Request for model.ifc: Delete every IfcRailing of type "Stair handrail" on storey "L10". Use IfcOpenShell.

First a look at what the model holds.

```python
import ifcopenshell
import ifcopenshell.util.element

model = ifcopenshell.open("model.ifc")
print(model.schema)
storey = next(s for s in model.by_type("IfcBuildingStorey") if s.Name == "L10")
railings = [e for e in ifcopenshell.util.element.get_decomposition(storey) if e.is_a("IfcRailing")]
seen = {}
for e in railings:
    element_type = ifcopenshell.util.element.get_type(e)
    name = element_type.Name if element_type not in (None, e) else None
    seen[name] = seen.get(name, 0) + 1
for name, count in sorted(seen.items(), key=str):
    print(count, "x", name)
```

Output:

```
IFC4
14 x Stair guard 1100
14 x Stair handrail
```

```python
import ifcopenshell
import ifcopenshell.api.root
import ifcopenshell.util.element

model = ifcopenshell.open("model.ifc")

storey = next(s for s in model.by_type("IfcBuildingStorey") if s.Name == "L10")
railings = [e for e in ifcopenshell.util.element.get_decomposition(storey) if e.is_a("IfcRailing")]
targets = [e for e in railings if (t := ifcopenshell.util.element.get_type(e)) not in (None, e) and t.Name == "Stair handrail"]

for e in targets:
    ifcopenshell.api.root.remove_product(model, product=e)
print(len(targets), "removed")

model.write("model_v2.ifc")
```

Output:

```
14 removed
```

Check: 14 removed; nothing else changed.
